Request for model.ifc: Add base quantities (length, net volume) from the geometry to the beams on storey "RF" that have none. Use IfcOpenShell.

First a look at what the model holds.

```python
import ifcopenshell
import ifcopenshell.util.element
import ifcopenshell.util.unit

model = ifcopenshell.open("model.ifc")
print(model.schema)
for unit_type in ("LENGTHUNIT", "AREAUNIT", "VOLUMEUNIT"):
    print(unit_type, ifcopenshell.util.unit.calculate_unit_scale(model, unit_type))
storey = next(s for s in model.by_type("IfcBuildingStorey") if s.Name == "RF")
beams = [e for e in ifcopenshell.util.element.get_decomposition(storey) if e.is_a("IfcBeam")]
for e in sorted(beams, key=lambda e: e.id()):
    print(e.id(), e.is_a(), e.Name, list(ifcopenshell.util.element.get_psets(e, qtos_only=True)), sep=" | ")
```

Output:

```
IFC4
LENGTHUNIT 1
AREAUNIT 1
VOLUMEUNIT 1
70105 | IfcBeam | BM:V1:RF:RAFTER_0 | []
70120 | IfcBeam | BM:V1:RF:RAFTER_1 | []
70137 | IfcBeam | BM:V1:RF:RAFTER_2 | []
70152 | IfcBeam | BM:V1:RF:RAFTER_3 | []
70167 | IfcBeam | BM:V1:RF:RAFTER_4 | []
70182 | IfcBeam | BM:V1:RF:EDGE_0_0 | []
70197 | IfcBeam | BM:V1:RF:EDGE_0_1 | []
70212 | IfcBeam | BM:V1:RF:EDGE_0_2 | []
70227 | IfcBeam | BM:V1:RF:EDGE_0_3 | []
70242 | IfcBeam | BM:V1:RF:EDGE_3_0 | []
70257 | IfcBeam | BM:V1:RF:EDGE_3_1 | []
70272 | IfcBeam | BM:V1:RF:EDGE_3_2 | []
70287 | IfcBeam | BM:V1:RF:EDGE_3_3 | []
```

```python
import ifcopenshell
import ifcopenshell.api.pset
import ifcopenshell.geom
import ifcopenshell.util.element
import ifcopenshell.util.shape
import ifcopenshell.util.unit

model = ifcopenshell.open("model.ifc")
unit_scale = ifcopenshell.util.unit.calculate_unit_scale(model)
volume_scale = ifcopenshell.util.unit.calculate_unit_scale(model, "VOLUMEUNIT")
settings = ifcopenshell.geom.settings()

storey = next(s for s in model.by_type("IfcBuildingStorey") if s.Name == "RF")
beams = [e for e in ifcopenshell.util.element.get_decomposition(storey) if e.is_a("IfcBeam")]

for e in sorted(beams, key=lambda e: e.id()):
    if ifcopenshell.util.element.get_psets(e, qtos_only=True, should_inherit=False):
        continue
    # Geometry comes back in metres, in the element's own axes.
    shape = ifcopenshell.geom.create_shape(settings, e)
    values = {
        "Length": ifcopenshell.util.shape.get_max_xyz(shape.geometry) / unit_scale,
        "NetVolume": ifcopenshell.util.shape.get_volume(shape.geometry) / volume_scale,
    }
    qto = ifcopenshell.api.pset.add_qto(model, product=e, name="Qto_BeamBaseQuantities")
    ifcopenshell.api.pset.edit_qto(model, qto=qto, properties=values)
    print(e.id(), {k: round(v, 3) for k, v in values.items()})

model.write("model_v2.ifc")
```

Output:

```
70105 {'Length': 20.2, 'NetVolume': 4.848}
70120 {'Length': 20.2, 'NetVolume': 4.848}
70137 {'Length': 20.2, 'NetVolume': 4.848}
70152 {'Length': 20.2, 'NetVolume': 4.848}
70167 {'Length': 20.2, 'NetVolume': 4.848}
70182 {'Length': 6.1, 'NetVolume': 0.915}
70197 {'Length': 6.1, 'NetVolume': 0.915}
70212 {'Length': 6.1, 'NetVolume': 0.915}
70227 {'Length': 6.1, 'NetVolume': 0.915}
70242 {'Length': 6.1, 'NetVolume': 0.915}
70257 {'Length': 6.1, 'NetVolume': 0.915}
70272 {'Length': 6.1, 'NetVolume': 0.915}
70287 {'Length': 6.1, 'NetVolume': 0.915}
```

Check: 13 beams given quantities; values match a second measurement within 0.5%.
